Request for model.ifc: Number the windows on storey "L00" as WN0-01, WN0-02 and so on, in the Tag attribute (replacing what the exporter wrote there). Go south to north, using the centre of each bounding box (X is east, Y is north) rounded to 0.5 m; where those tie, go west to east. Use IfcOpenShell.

First a look at what the model holds.

```python
import ifcopenshell
import ifcopenshell.util.element
import ifcopenshell.util.placement

model = ifcopenshell.open("model.ifc")
print(model.schema)
storey = next(s for s in model.by_type("IfcBuildingStorey") if s.Name == "L00")
windows = [e for e in ifcopenshell.util.element.get_decomposition(storey) if e.is_a("IfcWindow")]
for e in sorted(windows, key=lambda e: e.id()):
    origin = ifcopenshell.util.placement.get_local_placement(e.ObjectPlacement)[:3, 3]
    print(e.id(), e.Tag, e.Name, origin.round(2) + 0.0, sep=" | ")
```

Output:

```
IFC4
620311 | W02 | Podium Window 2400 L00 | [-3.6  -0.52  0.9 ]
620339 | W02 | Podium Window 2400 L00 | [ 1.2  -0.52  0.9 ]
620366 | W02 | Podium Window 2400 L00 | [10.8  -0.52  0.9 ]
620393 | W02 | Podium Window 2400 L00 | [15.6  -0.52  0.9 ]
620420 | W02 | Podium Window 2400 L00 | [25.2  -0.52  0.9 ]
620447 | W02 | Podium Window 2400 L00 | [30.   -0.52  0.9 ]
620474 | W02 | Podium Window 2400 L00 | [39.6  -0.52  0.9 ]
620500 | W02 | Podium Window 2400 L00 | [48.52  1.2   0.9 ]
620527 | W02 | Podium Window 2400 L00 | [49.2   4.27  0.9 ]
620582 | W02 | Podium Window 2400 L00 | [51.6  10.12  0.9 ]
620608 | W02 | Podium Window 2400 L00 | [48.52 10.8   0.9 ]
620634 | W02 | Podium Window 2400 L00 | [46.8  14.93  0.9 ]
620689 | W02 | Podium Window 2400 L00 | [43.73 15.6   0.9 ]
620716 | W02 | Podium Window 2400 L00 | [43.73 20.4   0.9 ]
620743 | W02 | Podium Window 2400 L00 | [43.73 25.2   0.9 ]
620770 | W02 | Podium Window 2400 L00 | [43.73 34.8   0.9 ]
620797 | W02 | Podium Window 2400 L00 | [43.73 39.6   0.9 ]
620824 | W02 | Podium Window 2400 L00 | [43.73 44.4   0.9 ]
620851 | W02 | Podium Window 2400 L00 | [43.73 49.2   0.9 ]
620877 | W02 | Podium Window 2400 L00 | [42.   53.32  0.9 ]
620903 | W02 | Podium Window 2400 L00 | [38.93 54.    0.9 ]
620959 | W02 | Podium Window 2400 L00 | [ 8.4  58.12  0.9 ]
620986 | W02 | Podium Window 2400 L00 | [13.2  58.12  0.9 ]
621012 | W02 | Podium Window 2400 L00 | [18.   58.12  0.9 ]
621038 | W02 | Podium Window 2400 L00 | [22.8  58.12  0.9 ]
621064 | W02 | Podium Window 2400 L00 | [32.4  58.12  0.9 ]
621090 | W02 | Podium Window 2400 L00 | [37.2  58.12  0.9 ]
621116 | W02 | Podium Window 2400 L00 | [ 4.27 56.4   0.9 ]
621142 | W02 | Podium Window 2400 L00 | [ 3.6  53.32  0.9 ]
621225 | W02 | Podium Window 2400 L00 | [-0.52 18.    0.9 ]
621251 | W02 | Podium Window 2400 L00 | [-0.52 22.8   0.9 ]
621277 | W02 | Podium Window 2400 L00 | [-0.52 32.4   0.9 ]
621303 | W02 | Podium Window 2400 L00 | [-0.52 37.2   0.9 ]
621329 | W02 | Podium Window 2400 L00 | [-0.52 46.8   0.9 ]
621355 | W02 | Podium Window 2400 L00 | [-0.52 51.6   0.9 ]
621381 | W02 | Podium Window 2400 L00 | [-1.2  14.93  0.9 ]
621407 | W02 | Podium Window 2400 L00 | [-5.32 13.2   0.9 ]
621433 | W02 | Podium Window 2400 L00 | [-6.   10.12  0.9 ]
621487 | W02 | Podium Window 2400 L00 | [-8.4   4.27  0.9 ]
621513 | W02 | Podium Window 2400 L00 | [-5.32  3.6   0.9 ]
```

```python
import ifcopenshell
import ifcopenshell.geom
import ifcopenshell.util.element
import ifcopenshell.util.shape

model = ifcopenshell.open("model.ifc")
settings = ifcopenshell.geom.settings()
settings.set("use-world-coords", True)


def centre(element):
    shape = ifcopenshell.geom.create_shape(settings, element)
    return ifcopenshell.util.shape.get_bbox_centroid(shape.geometry)


storey = next(s for s in model.by_type("IfcBuildingStorey") if s.Name == "L00")
windows = [e for e in ifcopenshell.util.element.get_decomposition(storey) if e.is_a("IfcWindow")]

# Insertion points can sit at a corner or the storey origin, so sort by the geometry (in metres).
centres = {e: centre(e) for e in windows}
windows.sort(key=lambda e: (round(centres[e][1] / 0.5), centres[e][0]))

for i, e in enumerate(windows, start=1):
    number = f"WN0-{i:02d}"
    e.Tag = number
    print(e.id(), number)

model.write("model_rev.ifc")
```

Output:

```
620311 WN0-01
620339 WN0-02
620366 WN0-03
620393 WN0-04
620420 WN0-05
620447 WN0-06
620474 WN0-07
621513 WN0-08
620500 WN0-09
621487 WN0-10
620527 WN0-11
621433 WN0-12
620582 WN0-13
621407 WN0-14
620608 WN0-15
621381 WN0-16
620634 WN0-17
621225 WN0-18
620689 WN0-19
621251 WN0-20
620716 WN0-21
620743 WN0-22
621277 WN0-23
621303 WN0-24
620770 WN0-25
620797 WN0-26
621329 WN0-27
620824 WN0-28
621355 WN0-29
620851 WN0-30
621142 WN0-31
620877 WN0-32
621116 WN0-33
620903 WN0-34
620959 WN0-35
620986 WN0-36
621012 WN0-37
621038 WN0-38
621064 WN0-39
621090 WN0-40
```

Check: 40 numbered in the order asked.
